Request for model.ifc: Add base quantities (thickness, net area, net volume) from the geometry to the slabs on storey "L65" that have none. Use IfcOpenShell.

First a look at what the model holds.

```python
import ifcopenshell
import ifcopenshell.util.element
import ifcopenshell.util.unit

model = ifcopenshell.open("model.ifc")
print(model.schema)
for unit_type in ("LENGTHUNIT", "AREAUNIT", "VOLUMEUNIT"):
    print(unit_type, ifcopenshell.util.unit.calculate_unit_scale(model, unit_type))
storey = next(s for s in model.by_type("IfcBuildingStorey") if s.Name == "L65")
slabs = [e for e in ifcopenshell.util.element.get_decomposition(storey) if e.is_a("IfcSlab")]
for e in sorted(slabs, key=lambda e: e.id()):
    print(e.id(), e.is_a(), e.Name, list(ifcopenshell.util.element.get_psets(e, qtos_only=True)), sep=" | ")
```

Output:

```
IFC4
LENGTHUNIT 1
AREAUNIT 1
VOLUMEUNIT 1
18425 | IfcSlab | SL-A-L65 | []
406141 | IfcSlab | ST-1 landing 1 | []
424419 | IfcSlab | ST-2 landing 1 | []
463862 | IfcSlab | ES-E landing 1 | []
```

```python
import ifcopenshell
import ifcopenshell.api.pset
import ifcopenshell.geom
import ifcopenshell.util.element
import ifcopenshell.util.shape
import ifcopenshell.util.unit

model = ifcopenshell.open("model.ifc")
unit_scale = ifcopenshell.util.unit.calculate_unit_scale(model)
area_scale = ifcopenshell.util.unit.calculate_unit_scale(model, "AREAUNIT")
volume_scale = ifcopenshell.util.unit.calculate_unit_scale(model, "VOLUMEUNIT")
settings = ifcopenshell.geom.settings()

storey = next(s for s in model.by_type("IfcBuildingStorey") if s.Name == "L65")
slabs = [e for e in ifcopenshell.util.element.get_decomposition(storey) if e.is_a("IfcSlab")]

for e in sorted(slabs, key=lambda e: e.id()):
    if ifcopenshell.util.element.get_psets(e, qtos_only=True, should_inherit=False):
        continue
    # Geometry comes back in metres, in the element's own axes.
    shape = ifcopenshell.geom.create_shape(settings, e)
    values = {
        "Width": ifcopenshell.util.shape.get_z(shape.geometry) / unit_scale,
        "NetArea": ifcopenshell.util.shape.get_footprint_area(shape.geometry) / area_scale,
        "NetVolume": ifcopenshell.util.shape.get_volume(shape.geometry) / volume_scale,
    }
    qto = ifcopenshell.api.pset.add_qto(model, product=e, name="Qto_SlabBaseQuantities")
    ifcopenshell.api.pset.edit_qto(model, qto=qto, properties=values)
    print(e.id(), {k: round(v, 3) for k, v in values.items()})

model.write("model_v2.ifc")
```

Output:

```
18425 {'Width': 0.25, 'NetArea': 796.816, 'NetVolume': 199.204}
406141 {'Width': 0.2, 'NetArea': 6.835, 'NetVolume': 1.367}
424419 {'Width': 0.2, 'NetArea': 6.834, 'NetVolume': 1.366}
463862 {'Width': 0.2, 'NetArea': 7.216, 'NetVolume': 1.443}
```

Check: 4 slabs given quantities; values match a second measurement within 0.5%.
